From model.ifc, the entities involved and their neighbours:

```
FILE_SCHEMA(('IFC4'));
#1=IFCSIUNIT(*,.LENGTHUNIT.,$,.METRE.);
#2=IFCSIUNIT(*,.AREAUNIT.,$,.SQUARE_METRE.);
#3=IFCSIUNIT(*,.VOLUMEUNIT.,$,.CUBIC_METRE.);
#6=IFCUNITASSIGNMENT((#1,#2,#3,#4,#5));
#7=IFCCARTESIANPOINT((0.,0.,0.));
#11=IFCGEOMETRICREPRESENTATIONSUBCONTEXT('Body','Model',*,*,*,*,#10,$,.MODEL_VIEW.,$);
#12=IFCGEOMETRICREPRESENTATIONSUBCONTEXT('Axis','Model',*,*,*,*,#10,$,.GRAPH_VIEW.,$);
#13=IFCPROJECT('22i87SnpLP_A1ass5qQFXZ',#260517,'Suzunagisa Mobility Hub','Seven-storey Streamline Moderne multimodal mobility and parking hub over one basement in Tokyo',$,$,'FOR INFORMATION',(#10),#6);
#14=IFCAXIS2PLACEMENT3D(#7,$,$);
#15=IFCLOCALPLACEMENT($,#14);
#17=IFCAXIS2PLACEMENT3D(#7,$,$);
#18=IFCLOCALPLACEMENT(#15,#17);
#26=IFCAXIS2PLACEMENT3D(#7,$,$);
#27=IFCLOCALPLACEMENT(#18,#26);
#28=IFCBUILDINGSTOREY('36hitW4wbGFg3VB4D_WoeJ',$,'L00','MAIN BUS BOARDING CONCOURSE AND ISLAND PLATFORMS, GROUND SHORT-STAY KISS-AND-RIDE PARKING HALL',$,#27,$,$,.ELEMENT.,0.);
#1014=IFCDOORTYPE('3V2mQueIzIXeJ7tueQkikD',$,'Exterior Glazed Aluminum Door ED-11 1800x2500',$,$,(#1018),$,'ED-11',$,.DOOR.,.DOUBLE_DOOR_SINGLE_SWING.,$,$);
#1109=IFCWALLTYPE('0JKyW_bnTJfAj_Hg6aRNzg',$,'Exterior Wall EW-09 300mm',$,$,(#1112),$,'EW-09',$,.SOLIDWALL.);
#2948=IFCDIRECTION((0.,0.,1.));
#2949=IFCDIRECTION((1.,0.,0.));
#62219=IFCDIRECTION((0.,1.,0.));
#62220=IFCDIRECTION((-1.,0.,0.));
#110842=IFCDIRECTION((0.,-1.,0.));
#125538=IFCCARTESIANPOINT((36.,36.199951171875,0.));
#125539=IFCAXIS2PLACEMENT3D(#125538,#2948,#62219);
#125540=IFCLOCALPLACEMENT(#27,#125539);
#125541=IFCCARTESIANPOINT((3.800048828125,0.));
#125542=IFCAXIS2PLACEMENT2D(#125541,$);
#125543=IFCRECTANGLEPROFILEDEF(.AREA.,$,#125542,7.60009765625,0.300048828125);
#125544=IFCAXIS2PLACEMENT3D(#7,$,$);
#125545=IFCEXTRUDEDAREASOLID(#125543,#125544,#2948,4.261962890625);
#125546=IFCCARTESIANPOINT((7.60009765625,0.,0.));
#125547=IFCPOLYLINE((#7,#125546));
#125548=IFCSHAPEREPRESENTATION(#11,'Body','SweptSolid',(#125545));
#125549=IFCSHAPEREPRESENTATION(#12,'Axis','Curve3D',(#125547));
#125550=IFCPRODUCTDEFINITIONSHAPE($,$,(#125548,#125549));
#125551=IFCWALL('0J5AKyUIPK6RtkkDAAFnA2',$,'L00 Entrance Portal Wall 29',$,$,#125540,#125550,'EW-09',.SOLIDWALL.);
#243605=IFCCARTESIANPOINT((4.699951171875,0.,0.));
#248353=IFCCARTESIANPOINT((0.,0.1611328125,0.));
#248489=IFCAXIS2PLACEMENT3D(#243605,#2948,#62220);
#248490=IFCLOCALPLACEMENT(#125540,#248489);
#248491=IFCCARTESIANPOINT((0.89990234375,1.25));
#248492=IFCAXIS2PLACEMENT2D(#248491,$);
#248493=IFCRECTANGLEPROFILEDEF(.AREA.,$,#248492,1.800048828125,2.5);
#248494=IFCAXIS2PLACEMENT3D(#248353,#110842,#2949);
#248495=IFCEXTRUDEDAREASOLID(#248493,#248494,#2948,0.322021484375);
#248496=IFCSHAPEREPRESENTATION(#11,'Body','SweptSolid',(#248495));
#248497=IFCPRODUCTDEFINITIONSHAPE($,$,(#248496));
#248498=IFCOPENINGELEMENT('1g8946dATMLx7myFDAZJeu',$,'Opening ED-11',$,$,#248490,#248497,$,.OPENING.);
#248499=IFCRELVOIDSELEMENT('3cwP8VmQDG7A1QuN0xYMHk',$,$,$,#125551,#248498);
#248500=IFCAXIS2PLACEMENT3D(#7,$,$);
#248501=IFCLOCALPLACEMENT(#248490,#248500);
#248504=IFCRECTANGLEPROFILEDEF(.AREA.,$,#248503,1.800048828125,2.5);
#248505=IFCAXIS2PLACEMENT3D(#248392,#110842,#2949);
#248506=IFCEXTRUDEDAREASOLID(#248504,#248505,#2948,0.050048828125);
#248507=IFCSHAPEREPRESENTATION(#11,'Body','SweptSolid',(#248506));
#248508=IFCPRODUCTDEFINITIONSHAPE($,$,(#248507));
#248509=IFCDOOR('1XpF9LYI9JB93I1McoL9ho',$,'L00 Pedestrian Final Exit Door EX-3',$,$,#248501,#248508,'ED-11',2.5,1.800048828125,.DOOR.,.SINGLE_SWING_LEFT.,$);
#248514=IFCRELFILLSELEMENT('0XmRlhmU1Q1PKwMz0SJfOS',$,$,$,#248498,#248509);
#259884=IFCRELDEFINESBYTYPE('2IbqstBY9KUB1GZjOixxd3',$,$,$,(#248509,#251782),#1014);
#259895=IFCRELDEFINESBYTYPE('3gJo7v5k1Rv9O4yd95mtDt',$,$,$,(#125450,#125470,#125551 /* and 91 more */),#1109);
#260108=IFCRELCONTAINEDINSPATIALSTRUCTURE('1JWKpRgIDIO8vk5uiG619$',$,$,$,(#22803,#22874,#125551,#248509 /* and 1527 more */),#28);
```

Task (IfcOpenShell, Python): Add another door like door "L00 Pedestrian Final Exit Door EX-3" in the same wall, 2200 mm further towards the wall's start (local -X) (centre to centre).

```python
import ifcopenshell
import ifcopenshell.api.feature
import ifcopenshell.api.geometry
import ifcopenshell.api.root
import ifcopenshell.geom
import ifcopenshell.util.element
import ifcopenshell.util.placement
import ifcopenshell.util.shape
import ifcopenshell.util.unit

model = ifcopenshell.open("model.ifc")
unit_scale = ifcopenshell.util.unit.calculate_unit_scale(model)
settings = ifcopenshell.geom.settings()


def volume(element):
    """Net volume in cubic metres, openings subtracted."""
    shape = ifcopenshell.geom.create_shape(settings, element)
    return ifcopenshell.util.shape.get_volume(shape.geometry)


door = model.by_guid("1XpF9LYI9JB93I1McoL9ho")
opening = door.FillsVoids[0].RelatingOpeningElement
wall = opening.VoidsElements[0].RelatingBuildingElement
before = volume(wall)
shift = ifcopenshell.util.placement.get_local_placement(wall.ObjectPlacement)[:3, 0] * -2.2 / unit_scale

# copy_class copies the void relationship, type, container and properties, but no geometry.
new_opening = ifcopenshell.api.root.copy_class(model, product=opening)
new_opening.Representation = ifcopenshell.util.element.copy_deep(
    model, opening.Representation, exclude=["IfcGeometricRepresentationContext", "IfcRepresentationMap"]
)
new_door = ifcopenshell.api.root.copy_class(model, product=door)
new_door.Representation = ifcopenshell.util.element.copy_deep(
    model, door.Representation, exclude=["IfcGeometricRepresentationContext", "IfcRepresentationMap"]
)
new_door.Tag = None
ifcopenshell.api.feature.add_filling(model, opening=new_opening, element=new_door)

for old, new in ((opening, new_opening), (door, new_door)):
    matrix = ifcopenshell.util.placement.get_local_placement(old.ObjectPlacement)
    matrix[:3, 3] += shift
    ifcopenshell.api.geometry.edit_object_placement(model, product=new, matrix=matrix, is_si=False)

after = volume(wall)

print(f"wall volume {before:.3f} -> {after:.3f} m3")

model.write("model_v2.ifc")
```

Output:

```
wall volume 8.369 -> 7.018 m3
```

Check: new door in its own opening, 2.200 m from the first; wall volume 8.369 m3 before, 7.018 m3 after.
